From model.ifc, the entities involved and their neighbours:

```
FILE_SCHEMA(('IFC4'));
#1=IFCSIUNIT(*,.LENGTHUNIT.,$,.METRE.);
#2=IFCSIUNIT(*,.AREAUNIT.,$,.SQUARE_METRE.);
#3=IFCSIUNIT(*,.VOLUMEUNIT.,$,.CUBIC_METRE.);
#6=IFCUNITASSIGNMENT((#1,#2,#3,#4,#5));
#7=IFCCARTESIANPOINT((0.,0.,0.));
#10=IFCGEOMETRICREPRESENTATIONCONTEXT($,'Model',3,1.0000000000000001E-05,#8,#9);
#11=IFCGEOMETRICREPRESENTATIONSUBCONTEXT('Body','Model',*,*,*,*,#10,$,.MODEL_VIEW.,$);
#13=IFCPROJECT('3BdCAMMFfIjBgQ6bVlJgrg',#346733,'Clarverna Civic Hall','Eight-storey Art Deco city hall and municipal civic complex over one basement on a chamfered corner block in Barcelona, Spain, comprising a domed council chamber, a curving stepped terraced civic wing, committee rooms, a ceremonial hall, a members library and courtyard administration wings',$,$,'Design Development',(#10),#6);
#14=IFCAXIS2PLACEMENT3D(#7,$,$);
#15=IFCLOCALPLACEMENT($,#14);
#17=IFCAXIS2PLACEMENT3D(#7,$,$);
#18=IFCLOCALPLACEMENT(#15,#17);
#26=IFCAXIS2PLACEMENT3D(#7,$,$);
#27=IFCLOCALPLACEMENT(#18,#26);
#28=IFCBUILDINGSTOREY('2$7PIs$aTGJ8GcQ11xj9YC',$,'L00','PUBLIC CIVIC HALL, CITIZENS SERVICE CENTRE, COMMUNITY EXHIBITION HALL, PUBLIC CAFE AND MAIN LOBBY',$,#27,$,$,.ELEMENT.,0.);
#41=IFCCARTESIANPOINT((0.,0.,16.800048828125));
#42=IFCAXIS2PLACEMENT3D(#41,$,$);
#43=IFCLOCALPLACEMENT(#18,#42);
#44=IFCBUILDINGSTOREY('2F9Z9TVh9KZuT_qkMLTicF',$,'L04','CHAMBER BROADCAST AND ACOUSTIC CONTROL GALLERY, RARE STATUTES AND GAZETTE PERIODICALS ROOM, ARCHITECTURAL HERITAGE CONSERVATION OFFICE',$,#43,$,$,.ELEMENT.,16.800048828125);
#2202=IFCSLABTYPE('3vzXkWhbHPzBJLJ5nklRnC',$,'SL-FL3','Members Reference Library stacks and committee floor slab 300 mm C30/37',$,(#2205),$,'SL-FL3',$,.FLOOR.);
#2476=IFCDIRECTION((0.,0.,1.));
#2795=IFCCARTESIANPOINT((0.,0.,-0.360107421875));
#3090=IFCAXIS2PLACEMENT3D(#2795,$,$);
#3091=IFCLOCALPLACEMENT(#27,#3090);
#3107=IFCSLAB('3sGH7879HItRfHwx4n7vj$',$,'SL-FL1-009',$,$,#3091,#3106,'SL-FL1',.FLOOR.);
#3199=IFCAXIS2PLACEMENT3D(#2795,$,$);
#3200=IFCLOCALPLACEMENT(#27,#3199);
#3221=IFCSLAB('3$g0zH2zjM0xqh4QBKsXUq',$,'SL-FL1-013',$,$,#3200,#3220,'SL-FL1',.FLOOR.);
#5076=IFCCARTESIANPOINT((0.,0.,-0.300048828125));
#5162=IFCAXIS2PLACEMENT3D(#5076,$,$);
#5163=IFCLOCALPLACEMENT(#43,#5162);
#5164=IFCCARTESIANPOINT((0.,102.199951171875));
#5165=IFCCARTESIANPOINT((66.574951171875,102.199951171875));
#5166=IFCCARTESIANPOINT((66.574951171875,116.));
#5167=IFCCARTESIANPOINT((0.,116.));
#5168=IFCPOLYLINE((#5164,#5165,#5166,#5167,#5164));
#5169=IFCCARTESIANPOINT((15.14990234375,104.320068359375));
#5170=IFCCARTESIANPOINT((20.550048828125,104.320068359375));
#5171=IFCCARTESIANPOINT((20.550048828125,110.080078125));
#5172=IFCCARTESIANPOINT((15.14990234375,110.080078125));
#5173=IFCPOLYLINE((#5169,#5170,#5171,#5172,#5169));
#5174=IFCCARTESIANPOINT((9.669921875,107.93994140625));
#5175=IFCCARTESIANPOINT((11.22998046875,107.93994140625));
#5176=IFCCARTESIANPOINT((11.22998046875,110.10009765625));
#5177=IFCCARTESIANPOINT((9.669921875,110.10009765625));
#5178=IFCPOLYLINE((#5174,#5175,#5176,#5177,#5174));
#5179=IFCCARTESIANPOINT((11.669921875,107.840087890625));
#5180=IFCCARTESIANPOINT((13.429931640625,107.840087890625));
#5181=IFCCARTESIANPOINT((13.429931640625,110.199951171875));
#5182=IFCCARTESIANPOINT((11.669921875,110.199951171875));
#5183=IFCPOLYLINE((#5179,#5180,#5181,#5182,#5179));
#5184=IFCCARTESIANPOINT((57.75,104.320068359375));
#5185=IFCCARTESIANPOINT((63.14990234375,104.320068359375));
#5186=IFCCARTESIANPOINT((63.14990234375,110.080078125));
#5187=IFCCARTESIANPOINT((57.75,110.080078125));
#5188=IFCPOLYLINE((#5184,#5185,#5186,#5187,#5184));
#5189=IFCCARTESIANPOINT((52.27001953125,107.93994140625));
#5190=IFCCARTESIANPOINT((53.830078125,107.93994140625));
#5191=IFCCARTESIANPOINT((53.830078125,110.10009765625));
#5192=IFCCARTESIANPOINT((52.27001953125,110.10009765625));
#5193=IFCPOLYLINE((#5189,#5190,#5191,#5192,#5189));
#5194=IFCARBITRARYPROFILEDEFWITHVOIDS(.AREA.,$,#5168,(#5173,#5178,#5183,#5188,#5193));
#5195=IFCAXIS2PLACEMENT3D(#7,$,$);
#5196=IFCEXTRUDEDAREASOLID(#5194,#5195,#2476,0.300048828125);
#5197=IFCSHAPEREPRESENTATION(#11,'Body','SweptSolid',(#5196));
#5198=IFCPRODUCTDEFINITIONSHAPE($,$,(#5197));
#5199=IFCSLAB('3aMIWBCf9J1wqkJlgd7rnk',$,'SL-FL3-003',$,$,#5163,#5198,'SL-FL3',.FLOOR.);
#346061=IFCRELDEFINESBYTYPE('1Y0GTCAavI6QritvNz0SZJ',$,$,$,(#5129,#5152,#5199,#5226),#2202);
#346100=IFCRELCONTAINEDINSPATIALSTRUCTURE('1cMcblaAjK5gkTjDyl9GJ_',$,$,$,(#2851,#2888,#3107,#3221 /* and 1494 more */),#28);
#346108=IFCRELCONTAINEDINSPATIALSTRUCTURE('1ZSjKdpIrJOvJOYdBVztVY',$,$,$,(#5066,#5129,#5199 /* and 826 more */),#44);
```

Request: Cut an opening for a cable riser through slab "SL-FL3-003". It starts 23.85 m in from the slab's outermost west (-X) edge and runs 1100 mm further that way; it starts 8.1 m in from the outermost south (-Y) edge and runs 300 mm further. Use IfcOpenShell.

```python
import numpy as np
import ifcopenshell
import ifcopenshell.api.feature
import ifcopenshell.api.geometry
import ifcopenshell.api.root
import ifcopenshell.geom
import ifcopenshell.util.placement
import ifcopenshell.util.representation
import ifcopenshell.util.shape
import ifcopenshell.util.unit

model = ifcopenshell.open("model.ifc")
unit_scale = ifcopenshell.util.unit.calculate_unit_scale(model)
settings = ifcopenshell.geom.settings()


def volume(element):
    """Net volume in cubic metres, openings subtracted."""
    shape = ifcopenshell.geom.create_shape(settings, element)
    return ifcopenshell.util.shape.get_volume(shape.geometry)


slab = model.by_guid("3aMIWBCf9J1wqkJlgd7rnk")
before = volume(slab)

# Extent in the slab's own axes, in metres. The edges named are its -X and -Y sides.
slab_shape = ifcopenshell.geom.create_shape(settings, slab)
vertices = ifcopenshell.util.shape.get_vertices(slab_shape.geometry)
x_min, y_min, bottom = vertices.min(axis=0)
top = vertices[:, 2].max()

opening = ifcopenshell.api.root.create_entity(model, ifc_class="IfcOpeningElement", name="Cable riser opening", predefined_type="OPENING")
context = ifcopenshell.util.representation.get_context(model, "Model", "Body", "MODEL_VIEW")
width, depth = 1.1, 0.3
outline = [(0.0, 0.0), (width, 0.0), (width, depth), (0.0, depth), (0.0, 0.0)]
# Overshoot both faces by 50 mm so the cut is clean.
shape = ifcopenshell.api.geometry.add_slab_representation(
    model, context=context, depth=top - bottom + 0.1, polyline=outline
)
ifcopenshell.api.geometry.assign_representation(model, product=opening, representation=shape)

matrix = ifcopenshell.util.placement.get_local_placement(slab.ObjectPlacement)
matrix[:, 3] = matrix @ np.append(np.array([x_min + 23.85, y_min + 8.1, bottom - 0.05]) / unit_scale, 1.0)
ifcopenshell.api.geometry.edit_object_placement(model, product=opening, matrix=matrix, is_si=False)
ifcopenshell.api.feature.add_feature(model, feature=opening, element=slab)

after = volume(slab)

print(f"slab volume {before:.3f} -> {after:.3f} m3")

model.write("model-out.ifc")
```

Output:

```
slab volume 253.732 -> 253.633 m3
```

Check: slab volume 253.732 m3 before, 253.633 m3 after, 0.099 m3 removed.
